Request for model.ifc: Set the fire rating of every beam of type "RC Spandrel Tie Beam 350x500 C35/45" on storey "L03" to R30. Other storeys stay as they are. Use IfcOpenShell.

First a look at what the model holds.

```python
import ifcopenshell
import ifcopenshell.util.element

model = ifcopenshell.open("model.ifc")
print(model.schema)
storey = next(s for s in model.by_type("IfcBuildingStorey") if s.Name == "L03")
beams = [e for e in ifcopenshell.util.element.get_decomposition(storey) if e.is_a("IfcBeam")]
seen = {}
for e in beams:
    element_type = ifcopenshell.util.element.get_type(e)
    key = (element_type.Name if element_type != e and element_type else None, ifcopenshell.util.element.get_pset(e, "Pset_BeamCommon", "FireRating"))
    seen[key] = seen.get(key, 0) + 1
for (name, value), count in sorted(seen.items(), key=str):
    print(count, "x", name, "|", value)
```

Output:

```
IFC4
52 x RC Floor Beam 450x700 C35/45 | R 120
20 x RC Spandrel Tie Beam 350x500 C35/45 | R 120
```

```python
import ifcopenshell
import ifcopenshell.api.pset
import ifcopenshell.util.element

model = ifcopenshell.open("model.ifc")

storey = next(s for s in model.by_type("IfcBuildingStorey") if s.Name == "L03")
beams = [e for e in ifcopenshell.util.element.get_decomposition(storey) if e.is_a("IfcBeam")]

count = 0
for e in beams:
    element_type = ifcopenshell.util.element.get_type(e)
    if element_type in (None, e) or element_type.Name != "RC Spandrel Tie Beam 350x500 C35/45":
        continue
    # add_pset returns the element's existing set when there is one.
    pset = ifcopenshell.api.pset.add_pset(model, product=e, name="Pset_BeamCommon")
    ifcopenshell.api.pset.edit_pset(model, pset=pset, properties={"FireRating": "R30"})
    count += 1

print(count, "beams updated")

model.write("model-out.ifc")
```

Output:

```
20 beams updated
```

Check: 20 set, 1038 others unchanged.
